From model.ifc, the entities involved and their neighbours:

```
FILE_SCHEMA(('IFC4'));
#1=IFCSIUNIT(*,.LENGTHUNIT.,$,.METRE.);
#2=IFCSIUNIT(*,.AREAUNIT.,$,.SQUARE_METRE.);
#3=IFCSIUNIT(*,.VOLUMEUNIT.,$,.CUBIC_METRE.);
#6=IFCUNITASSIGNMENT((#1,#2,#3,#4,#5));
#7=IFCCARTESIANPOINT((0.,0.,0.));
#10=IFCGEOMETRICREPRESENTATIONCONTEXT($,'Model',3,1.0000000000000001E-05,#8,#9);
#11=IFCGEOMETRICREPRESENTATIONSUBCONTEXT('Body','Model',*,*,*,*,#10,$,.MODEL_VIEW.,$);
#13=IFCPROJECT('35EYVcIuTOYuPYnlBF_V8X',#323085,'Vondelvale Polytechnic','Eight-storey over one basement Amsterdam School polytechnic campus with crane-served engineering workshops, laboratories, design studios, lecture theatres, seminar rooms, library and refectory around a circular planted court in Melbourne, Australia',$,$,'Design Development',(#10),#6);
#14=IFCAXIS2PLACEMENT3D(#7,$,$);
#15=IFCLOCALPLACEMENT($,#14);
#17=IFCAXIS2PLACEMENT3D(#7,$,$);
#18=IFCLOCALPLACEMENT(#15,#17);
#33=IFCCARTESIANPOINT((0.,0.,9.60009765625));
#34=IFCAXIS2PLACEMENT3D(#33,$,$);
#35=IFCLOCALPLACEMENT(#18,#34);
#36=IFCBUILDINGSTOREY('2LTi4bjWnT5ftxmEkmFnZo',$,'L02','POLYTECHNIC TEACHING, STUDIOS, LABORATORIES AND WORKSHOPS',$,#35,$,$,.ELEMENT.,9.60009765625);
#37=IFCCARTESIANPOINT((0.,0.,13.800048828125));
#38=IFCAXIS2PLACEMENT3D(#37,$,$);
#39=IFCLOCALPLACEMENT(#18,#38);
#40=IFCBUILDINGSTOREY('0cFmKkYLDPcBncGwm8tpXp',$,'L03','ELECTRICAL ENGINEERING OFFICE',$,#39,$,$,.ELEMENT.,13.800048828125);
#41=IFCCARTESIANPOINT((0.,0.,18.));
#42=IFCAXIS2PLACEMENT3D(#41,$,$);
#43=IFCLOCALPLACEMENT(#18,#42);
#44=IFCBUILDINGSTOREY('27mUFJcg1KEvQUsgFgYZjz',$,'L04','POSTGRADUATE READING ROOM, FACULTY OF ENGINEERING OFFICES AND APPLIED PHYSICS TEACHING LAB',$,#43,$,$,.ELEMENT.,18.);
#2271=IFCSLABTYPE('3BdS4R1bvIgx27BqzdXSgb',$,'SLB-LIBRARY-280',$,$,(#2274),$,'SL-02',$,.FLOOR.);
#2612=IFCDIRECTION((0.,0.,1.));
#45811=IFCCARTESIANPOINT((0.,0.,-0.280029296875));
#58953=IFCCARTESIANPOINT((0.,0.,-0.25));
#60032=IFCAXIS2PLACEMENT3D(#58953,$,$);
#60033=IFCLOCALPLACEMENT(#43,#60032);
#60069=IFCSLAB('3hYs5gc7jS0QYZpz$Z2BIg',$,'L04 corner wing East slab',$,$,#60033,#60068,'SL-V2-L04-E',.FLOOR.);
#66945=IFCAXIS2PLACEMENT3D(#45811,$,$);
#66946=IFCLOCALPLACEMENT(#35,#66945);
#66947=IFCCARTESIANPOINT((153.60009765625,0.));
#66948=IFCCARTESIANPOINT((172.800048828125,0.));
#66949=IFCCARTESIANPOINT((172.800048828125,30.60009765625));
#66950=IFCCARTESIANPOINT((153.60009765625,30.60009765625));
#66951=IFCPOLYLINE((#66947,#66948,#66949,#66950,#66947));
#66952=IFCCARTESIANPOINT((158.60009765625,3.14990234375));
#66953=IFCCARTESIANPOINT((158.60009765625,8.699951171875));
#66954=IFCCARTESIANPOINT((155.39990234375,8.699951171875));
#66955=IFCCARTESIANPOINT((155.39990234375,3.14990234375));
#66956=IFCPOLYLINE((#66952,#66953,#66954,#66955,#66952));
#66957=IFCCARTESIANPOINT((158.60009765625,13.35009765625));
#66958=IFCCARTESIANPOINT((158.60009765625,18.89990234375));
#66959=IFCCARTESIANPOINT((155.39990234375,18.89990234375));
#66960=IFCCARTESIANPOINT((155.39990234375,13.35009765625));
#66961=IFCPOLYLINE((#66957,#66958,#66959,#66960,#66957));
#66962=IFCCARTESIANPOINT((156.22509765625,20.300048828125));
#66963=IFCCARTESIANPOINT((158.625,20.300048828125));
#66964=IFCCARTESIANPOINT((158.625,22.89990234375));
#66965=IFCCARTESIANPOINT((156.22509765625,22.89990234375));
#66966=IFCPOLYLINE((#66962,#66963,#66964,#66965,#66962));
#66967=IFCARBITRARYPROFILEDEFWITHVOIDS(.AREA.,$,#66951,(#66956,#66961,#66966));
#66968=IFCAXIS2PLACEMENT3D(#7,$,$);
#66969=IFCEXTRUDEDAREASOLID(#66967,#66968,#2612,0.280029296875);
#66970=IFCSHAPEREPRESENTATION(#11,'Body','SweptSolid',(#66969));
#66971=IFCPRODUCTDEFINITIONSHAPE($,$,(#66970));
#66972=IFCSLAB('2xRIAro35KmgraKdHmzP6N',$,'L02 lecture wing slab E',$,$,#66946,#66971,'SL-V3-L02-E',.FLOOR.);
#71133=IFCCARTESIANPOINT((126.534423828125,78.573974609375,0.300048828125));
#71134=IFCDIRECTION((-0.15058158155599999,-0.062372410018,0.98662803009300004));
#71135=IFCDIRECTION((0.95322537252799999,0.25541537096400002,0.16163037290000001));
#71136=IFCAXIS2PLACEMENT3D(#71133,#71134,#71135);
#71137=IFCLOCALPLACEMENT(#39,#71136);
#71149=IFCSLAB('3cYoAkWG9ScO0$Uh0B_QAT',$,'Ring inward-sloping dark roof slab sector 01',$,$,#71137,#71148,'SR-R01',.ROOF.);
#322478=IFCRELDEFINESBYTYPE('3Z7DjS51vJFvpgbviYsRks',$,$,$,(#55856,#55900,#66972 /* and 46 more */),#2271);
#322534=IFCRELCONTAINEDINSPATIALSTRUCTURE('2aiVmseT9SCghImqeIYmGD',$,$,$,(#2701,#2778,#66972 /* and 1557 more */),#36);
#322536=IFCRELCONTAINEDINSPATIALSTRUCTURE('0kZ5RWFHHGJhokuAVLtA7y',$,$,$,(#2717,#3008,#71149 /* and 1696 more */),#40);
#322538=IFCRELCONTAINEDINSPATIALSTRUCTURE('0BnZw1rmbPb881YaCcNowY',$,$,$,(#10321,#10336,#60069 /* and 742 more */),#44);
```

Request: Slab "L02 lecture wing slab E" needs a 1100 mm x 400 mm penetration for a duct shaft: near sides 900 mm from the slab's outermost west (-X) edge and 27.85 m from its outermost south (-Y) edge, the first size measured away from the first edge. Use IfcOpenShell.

```python
import numpy as np
import ifcopenshell
import ifcopenshell.api.feature
import ifcopenshell.api.geometry
import ifcopenshell.api.root
import ifcopenshell.geom
import ifcopenshell.util.placement
import ifcopenshell.util.representation
import ifcopenshell.util.shape
import ifcopenshell.util.unit

model = ifcopenshell.open("model.ifc")
unit_scale = ifcopenshell.util.unit.calculate_unit_scale(model)
settings = ifcopenshell.geom.settings()


def volume(element):
    """Net volume in cubic metres, openings subtracted."""
    shape = ifcopenshell.geom.create_shape(settings, element)
    return ifcopenshell.util.shape.get_volume(shape.geometry)


slab = model.by_id(66972)
before = volume(slab)

# Extent in the slab's own axes, in metres. The edges named are its -X and -Y sides.
slab_shape = ifcopenshell.geom.create_shape(settings, slab)
vertices = ifcopenshell.util.shape.get_vertices(slab_shape.geometry)
x_min, y_min, bottom = vertices.min(axis=0)
top = vertices[:, 2].max()

opening = ifcopenshell.api.root.create_entity(model, ifc_class="IfcOpeningElement", name="Duct shaft opening", predefined_type="OPENING")
context = ifcopenshell.util.representation.get_context(model, "Model", "Body", "MODEL_VIEW")
width, depth = 1.1, 0.4
outline = [(0.0, 0.0), (width, 0.0), (width, depth), (0.0, depth), (0.0, 0.0)]
# Overshoot both faces by 50 mm so the cut is clean.
shape = ifcopenshell.api.geometry.add_slab_representation(
    model, context=context, depth=top - bottom + 0.1, polyline=outline
)
ifcopenshell.api.geometry.assign_representation(model, product=opening, representation=shape)

matrix = ifcopenshell.util.placement.get_local_placement(slab.ObjectPlacement)
matrix[:, 3] = matrix @ np.append(np.array([x_min + 0.9, y_min + 27.85, bottom - 0.05]) / unit_scale, 1.0)
ifcopenshell.api.geometry.edit_object_placement(model, product=opening, matrix=matrix, is_si=False)
ifcopenshell.api.feature.add_feature(model, feature=opening, element=slab)

after = volume(slab)

print(f"slab volume {before:.3f} -> {after:.3f} m3")

model.write("model-out.ifc")
```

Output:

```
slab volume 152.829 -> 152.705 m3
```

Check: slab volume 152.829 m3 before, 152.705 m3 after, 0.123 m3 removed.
